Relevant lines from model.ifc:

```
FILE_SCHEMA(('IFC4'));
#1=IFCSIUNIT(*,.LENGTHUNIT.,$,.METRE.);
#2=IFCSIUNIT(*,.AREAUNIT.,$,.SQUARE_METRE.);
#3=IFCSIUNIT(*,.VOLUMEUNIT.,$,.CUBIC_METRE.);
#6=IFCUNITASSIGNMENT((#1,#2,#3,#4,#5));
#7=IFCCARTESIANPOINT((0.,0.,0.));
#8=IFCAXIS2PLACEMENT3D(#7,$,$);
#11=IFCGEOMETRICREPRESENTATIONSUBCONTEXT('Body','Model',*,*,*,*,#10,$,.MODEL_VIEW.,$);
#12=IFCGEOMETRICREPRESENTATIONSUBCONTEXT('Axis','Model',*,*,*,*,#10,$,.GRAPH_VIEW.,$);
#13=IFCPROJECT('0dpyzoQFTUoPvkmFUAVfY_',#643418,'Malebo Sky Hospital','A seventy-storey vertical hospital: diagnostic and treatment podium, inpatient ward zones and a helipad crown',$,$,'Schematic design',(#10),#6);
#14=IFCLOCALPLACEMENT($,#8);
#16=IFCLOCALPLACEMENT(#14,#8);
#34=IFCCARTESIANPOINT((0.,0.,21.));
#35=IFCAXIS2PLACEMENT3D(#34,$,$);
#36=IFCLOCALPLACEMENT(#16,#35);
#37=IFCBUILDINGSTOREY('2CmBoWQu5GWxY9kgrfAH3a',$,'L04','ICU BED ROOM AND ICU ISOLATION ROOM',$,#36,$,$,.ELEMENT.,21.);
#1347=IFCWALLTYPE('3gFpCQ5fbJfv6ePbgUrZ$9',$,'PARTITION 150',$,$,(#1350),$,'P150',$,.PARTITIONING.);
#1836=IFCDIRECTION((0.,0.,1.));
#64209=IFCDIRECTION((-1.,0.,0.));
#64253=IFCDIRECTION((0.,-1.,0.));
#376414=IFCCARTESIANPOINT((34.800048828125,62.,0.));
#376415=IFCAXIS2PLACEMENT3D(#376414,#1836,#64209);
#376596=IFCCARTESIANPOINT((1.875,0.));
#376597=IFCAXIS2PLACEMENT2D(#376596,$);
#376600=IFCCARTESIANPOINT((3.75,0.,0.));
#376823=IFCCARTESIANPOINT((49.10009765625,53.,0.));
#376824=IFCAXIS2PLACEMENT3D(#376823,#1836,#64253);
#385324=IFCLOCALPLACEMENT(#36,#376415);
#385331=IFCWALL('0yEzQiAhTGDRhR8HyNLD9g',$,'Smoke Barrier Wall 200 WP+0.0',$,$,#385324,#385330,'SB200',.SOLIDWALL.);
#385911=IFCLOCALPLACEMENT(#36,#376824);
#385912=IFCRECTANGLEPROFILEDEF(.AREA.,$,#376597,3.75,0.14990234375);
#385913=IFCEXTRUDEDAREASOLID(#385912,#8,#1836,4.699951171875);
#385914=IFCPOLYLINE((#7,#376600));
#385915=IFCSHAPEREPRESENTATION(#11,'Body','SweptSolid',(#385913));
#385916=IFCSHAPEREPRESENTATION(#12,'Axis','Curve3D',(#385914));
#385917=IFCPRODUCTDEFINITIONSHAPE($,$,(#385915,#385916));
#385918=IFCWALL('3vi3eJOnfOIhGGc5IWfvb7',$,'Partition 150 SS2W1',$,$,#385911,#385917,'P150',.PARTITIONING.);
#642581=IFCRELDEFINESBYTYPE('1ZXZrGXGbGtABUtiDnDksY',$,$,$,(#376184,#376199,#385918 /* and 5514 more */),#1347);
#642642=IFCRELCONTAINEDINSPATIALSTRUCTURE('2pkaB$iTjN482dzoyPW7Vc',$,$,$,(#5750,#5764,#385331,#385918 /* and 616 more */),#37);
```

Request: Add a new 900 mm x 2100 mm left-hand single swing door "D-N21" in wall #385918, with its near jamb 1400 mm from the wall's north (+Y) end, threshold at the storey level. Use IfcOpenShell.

```python
import numpy as np
import ifcopenshell
import ifcopenshell.api.feature
import ifcopenshell.api.geometry
import ifcopenshell.api.root
import ifcopenshell.api.spatial
import ifcopenshell.geom
import ifcopenshell.util.element
import ifcopenshell.util.placement
import ifcopenshell.util.representation
import ifcopenshell.util.shape
import ifcopenshell.util.unit

model = ifcopenshell.open("model.ifc")
unit_scale = ifcopenshell.util.unit.calculate_unit_scale(model)
settings = ifcopenshell.geom.settings()


def volume(element):
    """Net volume in cubic metres, openings subtracted."""
    shape = ifcopenshell.geom.create_shape(settings, element)
    return ifcopenshell.util.shape.get_volume(shape.geometry)


wall = model.by_guid("3vi3eJOnfOIhGGc5IWfvb7")
storey = ifcopenshell.util.element.get_container(wall, ifc_class="IfcBuildingStorey")
context = ifcopenshell.util.representation.get_context(model, "Model", "Body", "MODEL_VIEW")
before = volume(wall)

width, height, from_end, sill = 0.9, 2.1, 1.4, 0.0  # metres

# The wall runs along its own X axis, and the end named is its -X end.
wall_shape = ifcopenshell.geom.create_shape(settings, wall)
x, y, z = ifcopenshell.util.shape.get_vertices(wall_shape.geometry).T
start = x.min() + from_end
face, thickness = float(y.min()), float(y.max() - y.min())
wall_matrix = ifcopenshell.util.placement.get_local_placement(wall.ObjectPlacement)
level = ifcopenshell.util.placement.get_local_placement(storey.ObjectPlacement)[2, 3]


def in_wall(x, y):
    """Placement at x, y metres in the wall's axes, at sill height."""
    matrix = wall_matrix.copy()
    matrix[:, 3] = wall_matrix @ np.array([x / unit_scale, y / unit_scale, 0.0, 1.0])
    matrix[2, 3] = level + sill / unit_scale
    return matrix


# Opening: a box that overshoots both wall faces by 50 mm.
opening = ifcopenshell.api.root.create_entity(model, ifc_class="IfcOpeningElement", predefined_type="OPENING")
box = ifcopenshell.api.geometry.add_wall_representation(
    model, context=context, length=width, height=height, thickness=thickness + 0.1
)
ifcopenshell.api.geometry.assign_representation(model, product=opening, representation=box)
ifcopenshell.api.geometry.edit_object_placement(model, product=opening, matrix=in_wall(start, face - 0.05), is_si=False)
ifcopenshell.api.feature.add_feature(model, feature=opening, element=wall)

door = ifcopenshell.api.root.create_entity(model, ifc_class="IfcDoor", name="D-N21", predefined_type="DOOR")
door.OverallWidth, door.OverallHeight = width / unit_scale, height / unit_scale
door.OperationType = "SINGLE_SWING_LEFT"
body = ifcopenshell.api.geometry.add_door_representation(
    model,
    context=context,
    overall_width=door.OverallWidth,
    overall_height=door.OverallHeight,
    operation_type="SINGLE_SWING_LEFT",
    lining_properties={"LiningDepth": thickness / unit_scale, "ThresholdDepth": thickness / unit_scale},
)
ifcopenshell.api.geometry.assign_representation(model, product=door, representation=body)
ifcopenshell.api.spatial.assign_container(model, products=[door], relating_structure=storey)
ifcopenshell.api.feature.add_filling(model, opening=opening, element=door)

# The lining spans the wall, so the door starts at the wall face.
ifcopenshell.api.geometry.edit_object_placement(model, product=door, matrix=in_wall(start, face), is_si=False)

after = volume(wall)

print(f"wall volume {before:.3f} -> {after:.3f} m3")

model.write("model_edited.ifc")
```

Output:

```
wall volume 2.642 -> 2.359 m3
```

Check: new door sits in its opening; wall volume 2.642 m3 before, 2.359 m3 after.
